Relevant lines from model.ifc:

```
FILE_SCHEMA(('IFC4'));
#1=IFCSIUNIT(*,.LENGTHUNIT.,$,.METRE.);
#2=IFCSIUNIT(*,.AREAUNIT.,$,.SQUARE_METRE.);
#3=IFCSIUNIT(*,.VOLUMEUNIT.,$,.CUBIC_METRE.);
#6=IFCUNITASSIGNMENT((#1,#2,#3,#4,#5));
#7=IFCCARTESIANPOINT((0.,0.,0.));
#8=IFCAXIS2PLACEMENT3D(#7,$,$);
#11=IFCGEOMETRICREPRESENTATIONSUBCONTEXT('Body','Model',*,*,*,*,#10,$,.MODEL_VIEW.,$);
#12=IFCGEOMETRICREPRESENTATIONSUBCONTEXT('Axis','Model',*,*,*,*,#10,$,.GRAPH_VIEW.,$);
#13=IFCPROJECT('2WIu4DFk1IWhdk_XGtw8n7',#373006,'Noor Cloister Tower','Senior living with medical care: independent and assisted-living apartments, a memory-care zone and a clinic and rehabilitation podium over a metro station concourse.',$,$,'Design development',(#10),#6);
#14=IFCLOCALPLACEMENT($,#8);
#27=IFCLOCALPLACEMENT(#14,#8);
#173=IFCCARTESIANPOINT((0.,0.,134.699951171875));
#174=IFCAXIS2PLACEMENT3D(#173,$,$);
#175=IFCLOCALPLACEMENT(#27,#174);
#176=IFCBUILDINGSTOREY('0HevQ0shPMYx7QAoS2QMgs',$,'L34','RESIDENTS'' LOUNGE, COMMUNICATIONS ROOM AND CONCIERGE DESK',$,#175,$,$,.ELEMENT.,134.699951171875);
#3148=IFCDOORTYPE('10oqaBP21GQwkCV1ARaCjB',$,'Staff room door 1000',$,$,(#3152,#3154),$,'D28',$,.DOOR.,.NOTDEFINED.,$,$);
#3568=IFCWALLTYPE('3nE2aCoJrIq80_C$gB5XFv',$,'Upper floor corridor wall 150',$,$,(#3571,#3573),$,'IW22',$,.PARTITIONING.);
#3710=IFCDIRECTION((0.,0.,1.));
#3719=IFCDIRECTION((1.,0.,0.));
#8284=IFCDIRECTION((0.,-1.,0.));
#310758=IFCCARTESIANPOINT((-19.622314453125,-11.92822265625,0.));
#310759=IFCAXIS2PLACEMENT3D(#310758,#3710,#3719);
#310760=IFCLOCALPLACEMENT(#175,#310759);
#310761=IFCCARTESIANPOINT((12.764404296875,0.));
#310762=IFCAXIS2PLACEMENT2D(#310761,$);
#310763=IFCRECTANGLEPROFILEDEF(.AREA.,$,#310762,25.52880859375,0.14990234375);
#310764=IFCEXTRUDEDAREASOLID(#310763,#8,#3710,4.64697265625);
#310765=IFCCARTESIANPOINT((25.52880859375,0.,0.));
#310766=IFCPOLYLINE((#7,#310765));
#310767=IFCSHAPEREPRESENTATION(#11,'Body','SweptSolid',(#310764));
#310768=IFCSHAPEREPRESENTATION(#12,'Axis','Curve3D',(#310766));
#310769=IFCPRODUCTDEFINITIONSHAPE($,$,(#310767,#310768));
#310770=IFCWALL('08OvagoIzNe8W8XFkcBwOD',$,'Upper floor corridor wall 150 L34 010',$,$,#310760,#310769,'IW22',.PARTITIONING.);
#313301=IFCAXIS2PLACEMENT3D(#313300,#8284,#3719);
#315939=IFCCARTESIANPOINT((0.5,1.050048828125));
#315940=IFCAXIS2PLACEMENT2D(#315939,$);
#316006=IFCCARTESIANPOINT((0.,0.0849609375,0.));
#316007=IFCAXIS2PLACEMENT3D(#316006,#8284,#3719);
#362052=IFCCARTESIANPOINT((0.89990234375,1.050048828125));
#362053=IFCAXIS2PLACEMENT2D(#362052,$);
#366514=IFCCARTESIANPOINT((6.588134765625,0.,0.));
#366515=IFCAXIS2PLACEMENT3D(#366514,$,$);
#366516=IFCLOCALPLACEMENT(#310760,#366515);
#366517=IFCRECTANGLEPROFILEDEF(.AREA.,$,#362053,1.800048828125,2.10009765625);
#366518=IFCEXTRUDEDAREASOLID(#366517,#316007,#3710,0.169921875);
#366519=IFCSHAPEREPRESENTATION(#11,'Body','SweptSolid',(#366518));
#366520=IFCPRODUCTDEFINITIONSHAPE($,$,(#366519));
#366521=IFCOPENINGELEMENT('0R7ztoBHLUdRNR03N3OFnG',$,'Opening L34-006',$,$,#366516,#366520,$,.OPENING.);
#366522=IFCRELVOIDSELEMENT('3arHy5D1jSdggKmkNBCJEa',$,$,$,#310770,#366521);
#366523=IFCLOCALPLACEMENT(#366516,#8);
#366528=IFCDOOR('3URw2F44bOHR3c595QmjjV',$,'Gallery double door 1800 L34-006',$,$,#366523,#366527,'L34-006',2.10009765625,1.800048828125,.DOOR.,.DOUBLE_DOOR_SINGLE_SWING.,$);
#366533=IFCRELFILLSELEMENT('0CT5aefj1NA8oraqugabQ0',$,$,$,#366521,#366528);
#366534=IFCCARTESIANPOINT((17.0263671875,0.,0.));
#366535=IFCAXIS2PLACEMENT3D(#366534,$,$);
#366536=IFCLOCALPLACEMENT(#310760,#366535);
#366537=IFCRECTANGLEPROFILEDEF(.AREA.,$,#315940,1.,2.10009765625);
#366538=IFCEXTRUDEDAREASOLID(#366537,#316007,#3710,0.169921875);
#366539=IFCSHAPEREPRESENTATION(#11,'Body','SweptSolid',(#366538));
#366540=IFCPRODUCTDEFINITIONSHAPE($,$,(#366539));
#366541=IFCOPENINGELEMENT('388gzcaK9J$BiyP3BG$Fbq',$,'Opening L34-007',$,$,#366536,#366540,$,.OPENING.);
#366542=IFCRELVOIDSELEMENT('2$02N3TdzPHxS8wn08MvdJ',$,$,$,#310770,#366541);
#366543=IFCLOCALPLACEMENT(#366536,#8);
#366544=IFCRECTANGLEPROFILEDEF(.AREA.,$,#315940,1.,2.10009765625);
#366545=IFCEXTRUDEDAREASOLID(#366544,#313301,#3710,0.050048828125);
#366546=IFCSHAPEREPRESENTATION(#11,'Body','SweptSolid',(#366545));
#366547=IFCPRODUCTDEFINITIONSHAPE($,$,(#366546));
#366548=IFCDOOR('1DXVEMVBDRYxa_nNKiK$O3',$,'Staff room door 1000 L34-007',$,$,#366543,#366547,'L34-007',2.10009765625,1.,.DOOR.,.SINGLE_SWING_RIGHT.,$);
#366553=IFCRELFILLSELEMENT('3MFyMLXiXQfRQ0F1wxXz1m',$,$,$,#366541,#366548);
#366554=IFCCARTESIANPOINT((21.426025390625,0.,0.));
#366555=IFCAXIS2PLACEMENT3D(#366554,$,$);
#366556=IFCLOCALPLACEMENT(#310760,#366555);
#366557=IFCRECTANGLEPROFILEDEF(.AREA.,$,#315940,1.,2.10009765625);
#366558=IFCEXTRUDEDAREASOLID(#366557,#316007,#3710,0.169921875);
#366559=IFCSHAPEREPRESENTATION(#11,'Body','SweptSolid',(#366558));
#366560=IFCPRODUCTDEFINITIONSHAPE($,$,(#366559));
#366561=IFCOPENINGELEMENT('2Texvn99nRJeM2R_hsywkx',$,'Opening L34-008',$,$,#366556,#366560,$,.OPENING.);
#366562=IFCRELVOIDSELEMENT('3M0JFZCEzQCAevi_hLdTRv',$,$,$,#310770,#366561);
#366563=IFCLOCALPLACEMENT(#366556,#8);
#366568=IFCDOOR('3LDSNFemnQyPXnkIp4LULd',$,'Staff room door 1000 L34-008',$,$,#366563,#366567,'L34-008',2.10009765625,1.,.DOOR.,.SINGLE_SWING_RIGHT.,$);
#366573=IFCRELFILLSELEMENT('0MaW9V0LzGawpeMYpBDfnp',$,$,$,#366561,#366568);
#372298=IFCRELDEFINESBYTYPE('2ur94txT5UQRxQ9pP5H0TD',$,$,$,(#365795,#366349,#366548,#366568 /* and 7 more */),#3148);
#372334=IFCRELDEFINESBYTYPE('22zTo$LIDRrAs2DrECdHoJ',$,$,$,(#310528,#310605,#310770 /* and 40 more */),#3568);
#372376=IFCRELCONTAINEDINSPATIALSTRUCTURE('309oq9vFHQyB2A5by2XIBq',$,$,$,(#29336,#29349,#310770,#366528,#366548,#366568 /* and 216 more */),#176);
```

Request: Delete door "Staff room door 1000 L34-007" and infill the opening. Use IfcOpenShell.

```python
import ifcopenshell
import ifcopenshell.api.feature
import ifcopenshell.api.root
import ifcopenshell.geom
import ifcopenshell.util.shape

model = ifcopenshell.open("model.ifc")
settings = ifcopenshell.geom.settings()


def volume(element):
    """Net volume in cubic metres, openings subtracted."""
    shape = ifcopenshell.geom.create_shape(settings, element)
    return ifcopenshell.util.shape.get_volume(shape.geometry)


door = model.by_id(366548)
opening = door.FillsVoids[0].RelatingOpeningElement
wall = opening.VoidsElements[0].RelatingBuildingElement
before = volume(wall)

ifcopenshell.api.root.remove_product(model, product=door)
ifcopenshell.api.feature.remove_feature(model, feature=opening)

after = volume(wall)

print(f"wall volume {before:.3f} -> {after:.3f} m3")

model.write("model-out.ifc")
```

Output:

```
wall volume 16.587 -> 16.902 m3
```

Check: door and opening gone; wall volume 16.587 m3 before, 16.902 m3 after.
